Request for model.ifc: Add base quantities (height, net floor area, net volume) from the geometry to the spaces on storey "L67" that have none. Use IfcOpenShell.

First a look at what the model holds.

```python
import ifcopenshell
import ifcopenshell.util.element
import ifcopenshell.util.unit

model = ifcopenshell.open("model.ifc")
print(model.schema)
for unit_type in ("LENGTHUNIT", "AREAUNIT", "VOLUMEUNIT"):
    print(unit_type, ifcopenshell.util.unit.calculate_unit_scale(model, unit_type))
storey = next(s for s in model.by_type("IfcBuildingStorey") if s.Name == "L67")
spaces = [e for e in ifcopenshell.util.element.get_decomposition(storey) if e.is_a("IfcSpace")]
for e in sorted(spaces, key=lambda e: e.id()):
    print(e.id(), e.is_a(), e.Name, list(ifcopenshell.util.element.get_psets(e, qtos_only=True)), sep=" | ")
```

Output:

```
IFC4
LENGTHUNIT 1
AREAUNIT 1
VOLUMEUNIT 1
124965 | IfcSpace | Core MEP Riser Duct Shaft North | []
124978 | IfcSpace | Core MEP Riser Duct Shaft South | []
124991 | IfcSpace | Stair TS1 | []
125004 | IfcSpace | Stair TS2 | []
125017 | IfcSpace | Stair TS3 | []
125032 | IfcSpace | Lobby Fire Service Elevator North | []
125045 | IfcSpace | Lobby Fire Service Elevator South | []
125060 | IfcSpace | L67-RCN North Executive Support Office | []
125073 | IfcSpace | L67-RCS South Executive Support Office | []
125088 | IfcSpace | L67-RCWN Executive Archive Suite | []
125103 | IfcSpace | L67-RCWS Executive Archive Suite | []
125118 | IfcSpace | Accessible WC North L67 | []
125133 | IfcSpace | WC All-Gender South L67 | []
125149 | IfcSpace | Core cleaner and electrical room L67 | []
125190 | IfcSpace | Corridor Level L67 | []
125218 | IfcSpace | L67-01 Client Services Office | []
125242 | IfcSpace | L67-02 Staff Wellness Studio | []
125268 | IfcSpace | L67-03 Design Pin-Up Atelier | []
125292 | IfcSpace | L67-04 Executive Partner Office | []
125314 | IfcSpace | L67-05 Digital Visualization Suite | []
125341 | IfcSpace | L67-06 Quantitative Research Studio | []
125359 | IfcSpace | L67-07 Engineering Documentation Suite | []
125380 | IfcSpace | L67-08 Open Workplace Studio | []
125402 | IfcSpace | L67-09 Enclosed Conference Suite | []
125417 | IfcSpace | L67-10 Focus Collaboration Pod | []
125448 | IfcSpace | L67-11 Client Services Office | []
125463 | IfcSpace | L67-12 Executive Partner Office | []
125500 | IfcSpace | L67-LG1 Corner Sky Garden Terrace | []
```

```python
import ifcopenshell
import ifcopenshell.api.pset
import ifcopenshell.geom
import ifcopenshell.util.element
import ifcopenshell.util.shape
import ifcopenshell.util.unit

model = ifcopenshell.open("model.ifc")
unit_scale = ifcopenshell.util.unit.calculate_unit_scale(model)
area_scale = ifcopenshell.util.unit.calculate_unit_scale(model, "AREAUNIT")
volume_scale = ifcopenshell.util.unit.calculate_unit_scale(model, "VOLUMEUNIT")
settings = ifcopenshell.geom.settings()

storey = next(s for s in model.by_type("IfcBuildingStorey") if s.Name == "L67")
spaces = [e for e in ifcopenshell.util.element.get_decomposition(storey) if e.is_a("IfcSpace")]

for e in sorted(spaces, key=lambda e: e.id()):
    if ifcopenshell.util.element.get_psets(e, qtos_only=True, should_inherit=False):
        continue
    # Geometry comes back in metres, in the element's own axes.
    shape = ifcopenshell.geom.create_shape(settings, e)
    values = {
        "Height": ifcopenshell.util.shape.get_z(shape.geometry) / unit_scale,
        "NetFloorArea": ifcopenshell.util.shape.get_footprint_area(shape.geometry) / area_scale,
        "NetVolume": ifcopenshell.util.shape.get_volume(shape.geometry) / volume_scale,
    }
    qto = ifcopenshell.api.pset.add_qto(model, product=e, name="Qto_SpaceBaseQuantities")
    ifcopenshell.api.pset.edit_qto(model, qto=qto, properties=values)
    print(e.id(), {k: round(v, 3) for k, v in values.items()})

model.write("model_rev.ifc")
```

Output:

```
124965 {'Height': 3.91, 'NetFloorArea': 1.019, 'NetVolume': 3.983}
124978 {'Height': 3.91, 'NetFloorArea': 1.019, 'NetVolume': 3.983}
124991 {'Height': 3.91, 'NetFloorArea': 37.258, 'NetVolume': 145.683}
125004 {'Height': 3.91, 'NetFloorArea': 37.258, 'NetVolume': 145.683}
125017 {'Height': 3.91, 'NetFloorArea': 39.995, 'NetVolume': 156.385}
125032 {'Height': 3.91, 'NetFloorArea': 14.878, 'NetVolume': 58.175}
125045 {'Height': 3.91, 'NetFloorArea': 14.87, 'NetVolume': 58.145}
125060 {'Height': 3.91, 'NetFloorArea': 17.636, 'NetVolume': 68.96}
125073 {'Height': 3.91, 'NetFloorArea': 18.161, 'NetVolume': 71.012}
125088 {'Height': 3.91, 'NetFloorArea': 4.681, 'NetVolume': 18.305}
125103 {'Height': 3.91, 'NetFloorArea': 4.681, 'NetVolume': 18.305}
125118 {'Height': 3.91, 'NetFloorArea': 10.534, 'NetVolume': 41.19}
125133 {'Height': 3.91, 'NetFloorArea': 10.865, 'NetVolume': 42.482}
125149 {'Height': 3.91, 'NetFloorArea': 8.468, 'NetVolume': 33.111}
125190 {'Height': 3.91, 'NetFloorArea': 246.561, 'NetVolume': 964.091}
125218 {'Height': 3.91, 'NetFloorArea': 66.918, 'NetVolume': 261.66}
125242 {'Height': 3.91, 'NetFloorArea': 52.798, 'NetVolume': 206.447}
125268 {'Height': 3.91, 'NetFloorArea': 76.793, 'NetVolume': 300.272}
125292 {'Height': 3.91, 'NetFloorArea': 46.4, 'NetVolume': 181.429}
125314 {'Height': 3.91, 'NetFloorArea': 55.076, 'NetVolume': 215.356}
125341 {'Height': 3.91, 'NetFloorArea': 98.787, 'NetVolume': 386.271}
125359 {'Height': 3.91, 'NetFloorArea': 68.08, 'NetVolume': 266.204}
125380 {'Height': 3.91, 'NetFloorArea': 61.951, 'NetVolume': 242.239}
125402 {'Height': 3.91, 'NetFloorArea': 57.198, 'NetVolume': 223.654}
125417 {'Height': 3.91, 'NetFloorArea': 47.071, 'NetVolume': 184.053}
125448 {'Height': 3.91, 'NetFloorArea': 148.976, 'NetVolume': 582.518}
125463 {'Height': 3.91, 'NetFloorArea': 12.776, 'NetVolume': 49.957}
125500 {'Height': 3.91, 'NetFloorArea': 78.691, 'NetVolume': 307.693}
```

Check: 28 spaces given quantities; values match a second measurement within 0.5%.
